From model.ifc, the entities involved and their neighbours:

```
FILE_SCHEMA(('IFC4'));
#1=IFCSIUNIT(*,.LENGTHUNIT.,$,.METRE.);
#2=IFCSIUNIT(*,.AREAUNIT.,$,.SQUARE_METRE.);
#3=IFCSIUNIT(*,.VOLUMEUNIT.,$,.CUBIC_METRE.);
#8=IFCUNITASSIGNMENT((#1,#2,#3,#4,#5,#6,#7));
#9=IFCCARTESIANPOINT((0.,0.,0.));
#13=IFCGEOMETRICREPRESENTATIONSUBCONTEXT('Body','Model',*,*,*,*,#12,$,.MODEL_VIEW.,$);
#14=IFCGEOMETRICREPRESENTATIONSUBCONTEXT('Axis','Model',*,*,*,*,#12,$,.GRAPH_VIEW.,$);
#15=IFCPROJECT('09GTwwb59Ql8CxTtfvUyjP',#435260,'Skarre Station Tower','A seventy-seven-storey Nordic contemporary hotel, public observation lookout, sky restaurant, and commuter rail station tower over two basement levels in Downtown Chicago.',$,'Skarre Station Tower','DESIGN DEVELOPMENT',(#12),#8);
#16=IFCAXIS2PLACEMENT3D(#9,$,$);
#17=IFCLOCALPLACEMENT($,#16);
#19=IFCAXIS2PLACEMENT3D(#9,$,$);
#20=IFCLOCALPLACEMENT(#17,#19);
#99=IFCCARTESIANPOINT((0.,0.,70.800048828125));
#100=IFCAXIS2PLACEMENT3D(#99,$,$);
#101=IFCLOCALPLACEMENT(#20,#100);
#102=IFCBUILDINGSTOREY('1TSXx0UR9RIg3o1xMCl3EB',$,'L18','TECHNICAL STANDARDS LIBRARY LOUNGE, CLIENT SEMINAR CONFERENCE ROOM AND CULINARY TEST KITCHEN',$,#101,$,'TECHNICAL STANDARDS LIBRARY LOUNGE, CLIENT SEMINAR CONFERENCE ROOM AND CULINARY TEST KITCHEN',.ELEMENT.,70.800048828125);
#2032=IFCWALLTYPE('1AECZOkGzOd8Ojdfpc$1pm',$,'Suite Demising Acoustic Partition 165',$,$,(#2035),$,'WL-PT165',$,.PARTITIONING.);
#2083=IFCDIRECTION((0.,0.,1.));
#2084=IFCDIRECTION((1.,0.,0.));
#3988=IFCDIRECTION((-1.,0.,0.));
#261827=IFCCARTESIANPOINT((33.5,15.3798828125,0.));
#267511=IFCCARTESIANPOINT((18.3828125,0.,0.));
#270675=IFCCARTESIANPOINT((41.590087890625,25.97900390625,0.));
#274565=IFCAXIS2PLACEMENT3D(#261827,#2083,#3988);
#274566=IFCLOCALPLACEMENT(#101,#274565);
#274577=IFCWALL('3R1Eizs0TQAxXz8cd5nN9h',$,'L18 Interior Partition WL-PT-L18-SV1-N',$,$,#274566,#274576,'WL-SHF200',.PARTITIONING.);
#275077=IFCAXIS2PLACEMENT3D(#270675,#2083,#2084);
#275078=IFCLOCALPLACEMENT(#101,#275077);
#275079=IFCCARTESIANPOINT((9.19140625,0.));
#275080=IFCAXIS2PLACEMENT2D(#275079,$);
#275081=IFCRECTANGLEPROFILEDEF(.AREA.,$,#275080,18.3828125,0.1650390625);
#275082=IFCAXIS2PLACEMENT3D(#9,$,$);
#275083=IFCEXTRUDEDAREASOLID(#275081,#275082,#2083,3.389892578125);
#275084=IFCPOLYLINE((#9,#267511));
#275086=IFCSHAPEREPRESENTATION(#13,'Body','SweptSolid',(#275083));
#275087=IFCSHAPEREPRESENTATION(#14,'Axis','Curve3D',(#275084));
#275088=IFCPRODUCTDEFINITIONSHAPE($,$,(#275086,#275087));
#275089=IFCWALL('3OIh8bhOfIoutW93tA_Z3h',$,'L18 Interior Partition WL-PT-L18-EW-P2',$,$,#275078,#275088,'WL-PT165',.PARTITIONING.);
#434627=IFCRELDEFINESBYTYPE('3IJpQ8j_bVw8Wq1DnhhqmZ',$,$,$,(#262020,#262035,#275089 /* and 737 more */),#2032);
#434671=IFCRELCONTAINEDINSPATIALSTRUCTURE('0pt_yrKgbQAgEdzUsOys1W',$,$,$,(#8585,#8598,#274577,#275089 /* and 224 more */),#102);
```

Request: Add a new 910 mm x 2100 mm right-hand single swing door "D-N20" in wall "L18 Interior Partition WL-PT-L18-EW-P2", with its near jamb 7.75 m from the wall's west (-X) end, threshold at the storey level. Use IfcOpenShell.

```python
import numpy as np
import ifcopenshell
import ifcopenshell.api.feature
import ifcopenshell.api.geometry
import ifcopenshell.api.root
import ifcopenshell.api.spatial
import ifcopenshell.geom
import ifcopenshell.util.element
import ifcopenshell.util.placement
import ifcopenshell.util.representation
import ifcopenshell.util.shape
import ifcopenshell.util.unit

model = ifcopenshell.open("model.ifc")
unit_scale = ifcopenshell.util.unit.calculate_unit_scale(model)
settings = ifcopenshell.geom.settings()


def volume(element):
    """Net volume in cubic metres, openings subtracted."""
    shape = ifcopenshell.geom.create_shape(settings, element)
    return ifcopenshell.util.shape.get_volume(shape.geometry)


wall = model.by_guid("3OIh8bhOfIoutW93tA_Z3h")
storey = ifcopenshell.util.element.get_container(wall, ifc_class="IfcBuildingStorey")
context = ifcopenshell.util.representation.get_context(model, "Model", "Body", "MODEL_VIEW")
before = volume(wall)

width, height, from_end, sill = 0.91, 2.1, 7.75, 0.0  # metres

# The wall runs along its own X axis, and the end named is its -X end.
wall_shape = ifcopenshell.geom.create_shape(settings, wall)
x, y, z = ifcopenshell.util.shape.get_vertices(wall_shape.geometry).T
start = x.min() + from_end
face, thickness = float(y.min()), float(y.max() - y.min())
wall_matrix = ifcopenshell.util.placement.get_local_placement(wall.ObjectPlacement)
level = ifcopenshell.util.placement.get_local_placement(storey.ObjectPlacement)[2, 3]


def in_wall(x, y):
    """Placement at x, y metres in the wall's axes, at sill height."""
    matrix = wall_matrix.copy()
    matrix[:, 3] = wall_matrix @ np.array([x / unit_scale, y / unit_scale, 0.0, 1.0])
    matrix[2, 3] = level + sill / unit_scale
    return matrix


# Opening: a box that overshoots both wall faces by 50 mm.
opening = ifcopenshell.api.root.create_entity(model, ifc_class="IfcOpeningElement", predefined_type="OPENING")
box = ifcopenshell.api.geometry.add_wall_representation(
    model, context=context, length=width, height=height, thickness=thickness + 0.1
)
ifcopenshell.api.geometry.assign_representation(model, product=opening, representation=box)
ifcopenshell.api.geometry.edit_object_placement(model, product=opening, matrix=in_wall(start, face - 0.05), is_si=False)
ifcopenshell.api.feature.add_feature(model, feature=opening, element=wall)

door = ifcopenshell.api.root.create_entity(model, ifc_class="IfcDoor", name="D-N20", predefined_type="DOOR")
door.OverallWidth, door.OverallHeight = width / unit_scale, height / unit_scale
door.OperationType = "SINGLE_SWING_RIGHT"
body = ifcopenshell.api.geometry.add_door_representation(
    model,
    context=context,
    overall_width=door.OverallWidth,
    overall_height=door.OverallHeight,
    operation_type="SINGLE_SWING_RIGHT",
    lining_properties={"LiningDepth": thickness / unit_scale, "ThresholdDepth": thickness / unit_scale},
)
ifcopenshell.api.geometry.assign_representation(model, product=door, representation=body)
ifcopenshell.api.spatial.assign_container(model, products=[door], relating_structure=storey)
ifcopenshell.api.feature.add_filling(model, opening=opening, element=door)

# The lining spans the wall, so the door starts at the wall face.
ifcopenshell.api.geometry.edit_object_placement(model, product=door, matrix=in_wall(start, face), is_si=False)

after = volume(wall)

print(f"wall volume {before:.3f} -> {after:.3f} m3")

model.write("model-out.ifc")
```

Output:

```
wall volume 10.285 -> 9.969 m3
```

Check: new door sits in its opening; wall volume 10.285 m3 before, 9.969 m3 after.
